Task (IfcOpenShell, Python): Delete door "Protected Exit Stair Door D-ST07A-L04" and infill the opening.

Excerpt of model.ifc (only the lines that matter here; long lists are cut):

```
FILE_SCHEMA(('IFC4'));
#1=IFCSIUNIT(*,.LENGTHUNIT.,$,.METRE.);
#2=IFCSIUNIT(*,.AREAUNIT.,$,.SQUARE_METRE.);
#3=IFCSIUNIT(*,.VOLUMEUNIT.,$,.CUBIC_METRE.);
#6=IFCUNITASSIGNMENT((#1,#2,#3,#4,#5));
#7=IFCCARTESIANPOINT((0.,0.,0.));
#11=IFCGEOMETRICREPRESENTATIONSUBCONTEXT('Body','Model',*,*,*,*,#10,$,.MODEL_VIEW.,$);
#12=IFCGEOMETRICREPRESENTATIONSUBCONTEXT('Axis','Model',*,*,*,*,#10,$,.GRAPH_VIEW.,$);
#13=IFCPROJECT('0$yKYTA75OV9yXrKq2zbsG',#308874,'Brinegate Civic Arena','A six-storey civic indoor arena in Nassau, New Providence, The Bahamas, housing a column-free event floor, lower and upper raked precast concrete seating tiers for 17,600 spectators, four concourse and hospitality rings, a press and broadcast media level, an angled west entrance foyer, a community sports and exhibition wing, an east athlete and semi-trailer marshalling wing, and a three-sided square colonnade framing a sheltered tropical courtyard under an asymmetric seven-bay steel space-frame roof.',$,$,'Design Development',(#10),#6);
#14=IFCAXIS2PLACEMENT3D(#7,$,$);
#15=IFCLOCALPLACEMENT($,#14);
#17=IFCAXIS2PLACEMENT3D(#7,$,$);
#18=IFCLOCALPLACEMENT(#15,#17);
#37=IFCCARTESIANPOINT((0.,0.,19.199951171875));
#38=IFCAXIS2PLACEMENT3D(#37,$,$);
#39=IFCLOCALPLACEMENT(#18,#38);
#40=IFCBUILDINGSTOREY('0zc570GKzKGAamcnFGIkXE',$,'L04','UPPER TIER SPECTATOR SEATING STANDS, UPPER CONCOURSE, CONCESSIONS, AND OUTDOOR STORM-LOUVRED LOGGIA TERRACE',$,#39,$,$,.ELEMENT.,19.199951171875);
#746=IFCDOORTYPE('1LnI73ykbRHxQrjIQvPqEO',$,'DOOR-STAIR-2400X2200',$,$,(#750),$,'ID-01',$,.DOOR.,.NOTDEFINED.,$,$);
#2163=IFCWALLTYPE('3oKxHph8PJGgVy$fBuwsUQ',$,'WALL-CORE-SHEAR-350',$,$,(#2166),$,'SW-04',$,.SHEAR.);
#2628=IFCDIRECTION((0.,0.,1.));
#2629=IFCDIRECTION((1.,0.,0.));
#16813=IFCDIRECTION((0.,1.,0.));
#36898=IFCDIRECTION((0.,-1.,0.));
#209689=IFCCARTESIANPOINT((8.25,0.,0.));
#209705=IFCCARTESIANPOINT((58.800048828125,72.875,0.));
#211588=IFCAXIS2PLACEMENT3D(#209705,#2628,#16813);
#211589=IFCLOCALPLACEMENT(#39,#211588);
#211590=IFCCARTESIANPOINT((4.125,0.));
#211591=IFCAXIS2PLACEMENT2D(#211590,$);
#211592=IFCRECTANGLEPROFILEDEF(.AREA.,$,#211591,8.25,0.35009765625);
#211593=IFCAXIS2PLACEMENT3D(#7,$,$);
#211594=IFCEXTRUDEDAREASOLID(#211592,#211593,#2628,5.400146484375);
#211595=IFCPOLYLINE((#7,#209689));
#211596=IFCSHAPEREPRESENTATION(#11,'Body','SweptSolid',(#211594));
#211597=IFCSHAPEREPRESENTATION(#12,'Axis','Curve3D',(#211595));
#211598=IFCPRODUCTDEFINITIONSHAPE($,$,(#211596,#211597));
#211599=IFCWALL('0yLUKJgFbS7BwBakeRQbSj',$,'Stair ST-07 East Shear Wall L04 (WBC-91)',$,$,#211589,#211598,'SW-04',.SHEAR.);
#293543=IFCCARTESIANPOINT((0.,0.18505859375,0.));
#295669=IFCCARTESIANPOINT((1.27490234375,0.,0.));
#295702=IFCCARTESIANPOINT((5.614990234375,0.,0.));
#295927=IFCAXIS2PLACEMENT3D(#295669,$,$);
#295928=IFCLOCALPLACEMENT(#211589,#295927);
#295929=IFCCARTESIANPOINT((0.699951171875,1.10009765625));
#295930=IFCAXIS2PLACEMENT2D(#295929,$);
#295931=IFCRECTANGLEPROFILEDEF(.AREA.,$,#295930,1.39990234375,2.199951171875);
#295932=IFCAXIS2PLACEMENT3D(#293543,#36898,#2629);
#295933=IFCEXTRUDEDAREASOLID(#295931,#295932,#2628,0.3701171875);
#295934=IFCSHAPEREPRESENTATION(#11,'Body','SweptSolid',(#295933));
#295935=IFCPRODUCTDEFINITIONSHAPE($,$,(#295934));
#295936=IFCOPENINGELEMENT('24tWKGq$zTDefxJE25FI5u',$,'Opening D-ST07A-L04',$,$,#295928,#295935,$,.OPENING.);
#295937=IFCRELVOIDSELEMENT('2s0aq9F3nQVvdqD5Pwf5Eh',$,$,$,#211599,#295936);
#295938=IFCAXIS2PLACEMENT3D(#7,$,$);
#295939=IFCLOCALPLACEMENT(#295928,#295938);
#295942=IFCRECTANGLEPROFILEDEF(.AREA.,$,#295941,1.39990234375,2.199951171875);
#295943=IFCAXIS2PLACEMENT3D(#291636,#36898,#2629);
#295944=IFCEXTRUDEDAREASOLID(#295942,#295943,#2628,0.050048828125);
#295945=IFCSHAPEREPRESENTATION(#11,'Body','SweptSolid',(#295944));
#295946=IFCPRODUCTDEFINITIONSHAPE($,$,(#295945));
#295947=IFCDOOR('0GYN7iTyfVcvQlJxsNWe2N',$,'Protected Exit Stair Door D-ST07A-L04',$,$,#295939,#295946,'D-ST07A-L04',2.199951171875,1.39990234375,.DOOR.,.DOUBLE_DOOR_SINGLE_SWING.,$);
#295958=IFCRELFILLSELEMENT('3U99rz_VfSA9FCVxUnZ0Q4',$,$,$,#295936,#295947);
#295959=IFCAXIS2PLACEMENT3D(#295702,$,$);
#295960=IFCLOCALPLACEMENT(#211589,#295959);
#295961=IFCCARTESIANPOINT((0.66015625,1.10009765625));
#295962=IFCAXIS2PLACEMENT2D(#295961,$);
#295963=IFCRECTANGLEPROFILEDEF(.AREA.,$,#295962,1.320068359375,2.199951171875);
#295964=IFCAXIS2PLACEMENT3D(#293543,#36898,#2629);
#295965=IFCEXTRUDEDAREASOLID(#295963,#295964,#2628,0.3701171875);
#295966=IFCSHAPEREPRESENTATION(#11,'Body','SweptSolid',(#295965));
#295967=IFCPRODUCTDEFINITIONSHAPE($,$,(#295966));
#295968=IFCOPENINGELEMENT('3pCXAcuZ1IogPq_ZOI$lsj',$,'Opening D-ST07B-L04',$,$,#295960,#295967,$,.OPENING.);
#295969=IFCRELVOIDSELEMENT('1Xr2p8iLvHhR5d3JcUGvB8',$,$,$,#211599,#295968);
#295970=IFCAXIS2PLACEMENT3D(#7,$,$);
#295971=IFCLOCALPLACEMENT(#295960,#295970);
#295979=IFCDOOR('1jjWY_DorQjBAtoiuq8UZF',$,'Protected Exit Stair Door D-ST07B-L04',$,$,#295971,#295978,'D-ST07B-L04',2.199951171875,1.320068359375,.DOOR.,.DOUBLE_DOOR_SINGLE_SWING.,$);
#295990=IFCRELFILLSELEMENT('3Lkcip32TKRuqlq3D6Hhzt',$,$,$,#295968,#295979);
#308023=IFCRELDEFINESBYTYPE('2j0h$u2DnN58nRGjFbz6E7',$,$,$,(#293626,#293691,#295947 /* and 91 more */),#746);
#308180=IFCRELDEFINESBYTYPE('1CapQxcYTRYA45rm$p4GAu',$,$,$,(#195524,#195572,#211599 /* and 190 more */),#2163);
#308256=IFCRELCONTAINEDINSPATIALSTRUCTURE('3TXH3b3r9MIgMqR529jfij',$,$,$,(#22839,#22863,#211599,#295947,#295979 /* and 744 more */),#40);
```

```python
import ifcopenshell
import ifcopenshell.api.feature
import ifcopenshell.api.root
import ifcopenshell.geom
import ifcopenshell.util.shape

model = ifcopenshell.open("model.ifc")
settings = ifcopenshell.geom.settings()


def volume(element):
    """Net volume in cubic metres, openings subtracted."""
    shape = ifcopenshell.geom.create_shape(settings, element)
    return ifcopenshell.util.shape.get_volume(shape.geometry)


door = model.by_guid("0GYN7iTyfVcvQlJxsNWe2N")
opening = door.FillsVoids[0].RelatingOpeningElement
wall = opening.VoidsElements[0].RelatingBuildingElement
before = volume(wall)

ifcopenshell.api.root.remove_product(model, product=door)
ifcopenshell.api.feature.remove_feature(model, feature=opening)

after = volume(wall)

print(f"wall volume {before:.3f} -> {after:.3f} m3")

model.write("model_edited.ifc")
```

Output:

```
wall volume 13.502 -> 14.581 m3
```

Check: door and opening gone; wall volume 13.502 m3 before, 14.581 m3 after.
